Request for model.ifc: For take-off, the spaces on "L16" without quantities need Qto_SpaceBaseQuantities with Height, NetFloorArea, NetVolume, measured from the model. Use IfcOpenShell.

First a look at what the model holds.

```python
import ifcopenshell
import ifcopenshell.util.element
import ifcopenshell.util.unit

model = ifcopenshell.open("model.ifc")
print(model.schema)
for unit_type in ("LENGTHUNIT", "AREAUNIT", "VOLUMEUNIT"):
    print(unit_type, ifcopenshell.util.unit.calculate_unit_scale(model, unit_type))
storey = next(s for s in model.by_type("IfcBuildingStorey") if s.Name == "L16")
spaces = [e for e in ifcopenshell.util.element.get_decomposition(storey) if e.is_a("IfcSpace")]
for e in sorted(spaces, key=lambda e: e.id()):
    print(e.id(), e.is_a(), e.Name, list(ifcopenshell.util.element.get_psets(e, qtos_only=True)), sep=" | ")
```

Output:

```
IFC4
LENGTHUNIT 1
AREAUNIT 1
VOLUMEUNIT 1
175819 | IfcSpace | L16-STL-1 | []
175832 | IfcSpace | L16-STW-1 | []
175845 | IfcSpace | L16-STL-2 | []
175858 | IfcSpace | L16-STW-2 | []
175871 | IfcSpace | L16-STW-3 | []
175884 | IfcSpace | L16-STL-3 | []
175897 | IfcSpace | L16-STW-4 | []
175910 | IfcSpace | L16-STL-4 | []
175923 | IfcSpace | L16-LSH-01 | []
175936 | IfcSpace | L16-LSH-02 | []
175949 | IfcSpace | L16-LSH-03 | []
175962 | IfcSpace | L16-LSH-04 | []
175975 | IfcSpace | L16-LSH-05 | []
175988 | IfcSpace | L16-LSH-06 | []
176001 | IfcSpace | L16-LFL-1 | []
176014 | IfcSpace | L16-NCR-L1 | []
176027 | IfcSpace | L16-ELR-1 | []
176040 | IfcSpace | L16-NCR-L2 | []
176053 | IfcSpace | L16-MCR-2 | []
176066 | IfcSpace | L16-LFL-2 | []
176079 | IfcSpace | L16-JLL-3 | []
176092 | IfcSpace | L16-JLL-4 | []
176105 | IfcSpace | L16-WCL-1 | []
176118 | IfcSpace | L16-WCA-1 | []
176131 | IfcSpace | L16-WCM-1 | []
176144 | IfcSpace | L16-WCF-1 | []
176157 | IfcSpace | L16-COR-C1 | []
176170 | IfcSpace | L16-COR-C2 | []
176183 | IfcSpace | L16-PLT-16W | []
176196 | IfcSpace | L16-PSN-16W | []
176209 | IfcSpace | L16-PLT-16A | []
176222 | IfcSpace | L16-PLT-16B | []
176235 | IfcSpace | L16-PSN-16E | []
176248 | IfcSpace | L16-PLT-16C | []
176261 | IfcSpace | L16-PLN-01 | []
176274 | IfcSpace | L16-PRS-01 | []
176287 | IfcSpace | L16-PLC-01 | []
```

```python
import ifcopenshell
import ifcopenshell.api.pset
import ifcopenshell.geom
import ifcopenshell.util.element
import ifcopenshell.util.shape
import ifcopenshell.util.unit

model = ifcopenshell.open("model.ifc")
unit_scale = ifcopenshell.util.unit.calculate_unit_scale(model)
area_scale = ifcopenshell.util.unit.calculate_unit_scale(model, "AREAUNIT")
volume_scale = ifcopenshell.util.unit.calculate_unit_scale(model, "VOLUMEUNIT")
settings = ifcopenshell.geom.settings()

storey = next(s for s in model.by_type("IfcBuildingStorey") if s.Name == "L16")
spaces = [e for e in ifcopenshell.util.element.get_decomposition(storey) if e.is_a("IfcSpace")]

for e in sorted(spaces, key=lambda e: e.id()):
    if ifcopenshell.util.element.get_psets(e, qtos_only=True, should_inherit=False):
        continue
    # Geometry comes back in metres, in the element's own axes.
    shape = ifcopenshell.geom.create_shape(settings, e)
    values = {
        "Height": ifcopenshell.util.shape.get_z(shape.geometry) / unit_scale,
        "NetFloorArea": ifcopenshell.util.shape.get_footprint_area(shape.geometry) / area_scale,
        "NetVolume": ifcopenshell.util.shape.get_volume(shape.geometry) / volume_scale,
    }
    qto = ifcopenshell.api.pset.add_qto(model, product=e, name="Qto_SpaceBaseQuantities")
    ifcopenshell.api.pset.edit_qto(model, qto=qto, properties=values)
    print(e.id(), {k: round(v, 3) for k, v in values.items()})

model.write("model_v2.ifc")
```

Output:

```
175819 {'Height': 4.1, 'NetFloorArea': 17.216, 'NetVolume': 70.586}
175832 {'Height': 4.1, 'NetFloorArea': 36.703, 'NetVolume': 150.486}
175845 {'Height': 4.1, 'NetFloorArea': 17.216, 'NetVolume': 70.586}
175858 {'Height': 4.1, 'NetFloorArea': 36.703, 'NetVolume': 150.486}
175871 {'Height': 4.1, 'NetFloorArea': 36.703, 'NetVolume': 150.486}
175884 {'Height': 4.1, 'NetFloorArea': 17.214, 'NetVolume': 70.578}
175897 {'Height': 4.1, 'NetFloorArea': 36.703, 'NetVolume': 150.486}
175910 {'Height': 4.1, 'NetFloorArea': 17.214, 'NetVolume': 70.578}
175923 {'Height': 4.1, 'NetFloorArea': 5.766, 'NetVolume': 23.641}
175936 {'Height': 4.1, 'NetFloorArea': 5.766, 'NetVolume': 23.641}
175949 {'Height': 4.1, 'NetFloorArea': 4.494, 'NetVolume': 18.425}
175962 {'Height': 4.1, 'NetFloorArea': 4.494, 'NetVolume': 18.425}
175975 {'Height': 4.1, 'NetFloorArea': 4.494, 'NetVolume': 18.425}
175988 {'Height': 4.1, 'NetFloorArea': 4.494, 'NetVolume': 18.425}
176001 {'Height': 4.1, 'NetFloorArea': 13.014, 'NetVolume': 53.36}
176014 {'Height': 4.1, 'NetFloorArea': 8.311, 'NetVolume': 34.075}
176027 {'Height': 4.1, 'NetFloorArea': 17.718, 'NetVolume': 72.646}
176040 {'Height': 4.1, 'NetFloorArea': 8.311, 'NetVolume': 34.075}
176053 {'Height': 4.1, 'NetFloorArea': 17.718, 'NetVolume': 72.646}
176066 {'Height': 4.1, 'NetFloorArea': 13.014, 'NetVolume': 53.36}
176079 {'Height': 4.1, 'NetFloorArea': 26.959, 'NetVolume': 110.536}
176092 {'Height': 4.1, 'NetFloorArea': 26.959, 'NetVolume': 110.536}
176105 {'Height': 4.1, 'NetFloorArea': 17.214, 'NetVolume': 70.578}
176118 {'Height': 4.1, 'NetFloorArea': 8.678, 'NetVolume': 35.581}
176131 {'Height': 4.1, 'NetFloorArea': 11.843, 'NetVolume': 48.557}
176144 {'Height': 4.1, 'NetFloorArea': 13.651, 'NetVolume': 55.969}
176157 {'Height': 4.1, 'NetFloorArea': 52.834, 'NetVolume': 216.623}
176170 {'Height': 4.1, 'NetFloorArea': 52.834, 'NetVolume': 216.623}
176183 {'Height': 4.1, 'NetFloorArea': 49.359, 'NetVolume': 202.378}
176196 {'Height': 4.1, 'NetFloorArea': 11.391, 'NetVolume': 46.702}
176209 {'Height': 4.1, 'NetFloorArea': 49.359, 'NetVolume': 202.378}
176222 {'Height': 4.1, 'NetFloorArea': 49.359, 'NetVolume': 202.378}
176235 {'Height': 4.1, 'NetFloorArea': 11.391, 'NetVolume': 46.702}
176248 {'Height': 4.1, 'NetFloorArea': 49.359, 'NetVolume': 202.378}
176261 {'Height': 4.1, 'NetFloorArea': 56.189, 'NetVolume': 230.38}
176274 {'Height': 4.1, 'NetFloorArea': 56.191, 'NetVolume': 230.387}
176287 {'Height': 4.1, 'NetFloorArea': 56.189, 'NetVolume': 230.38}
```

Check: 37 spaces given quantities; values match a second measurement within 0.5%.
